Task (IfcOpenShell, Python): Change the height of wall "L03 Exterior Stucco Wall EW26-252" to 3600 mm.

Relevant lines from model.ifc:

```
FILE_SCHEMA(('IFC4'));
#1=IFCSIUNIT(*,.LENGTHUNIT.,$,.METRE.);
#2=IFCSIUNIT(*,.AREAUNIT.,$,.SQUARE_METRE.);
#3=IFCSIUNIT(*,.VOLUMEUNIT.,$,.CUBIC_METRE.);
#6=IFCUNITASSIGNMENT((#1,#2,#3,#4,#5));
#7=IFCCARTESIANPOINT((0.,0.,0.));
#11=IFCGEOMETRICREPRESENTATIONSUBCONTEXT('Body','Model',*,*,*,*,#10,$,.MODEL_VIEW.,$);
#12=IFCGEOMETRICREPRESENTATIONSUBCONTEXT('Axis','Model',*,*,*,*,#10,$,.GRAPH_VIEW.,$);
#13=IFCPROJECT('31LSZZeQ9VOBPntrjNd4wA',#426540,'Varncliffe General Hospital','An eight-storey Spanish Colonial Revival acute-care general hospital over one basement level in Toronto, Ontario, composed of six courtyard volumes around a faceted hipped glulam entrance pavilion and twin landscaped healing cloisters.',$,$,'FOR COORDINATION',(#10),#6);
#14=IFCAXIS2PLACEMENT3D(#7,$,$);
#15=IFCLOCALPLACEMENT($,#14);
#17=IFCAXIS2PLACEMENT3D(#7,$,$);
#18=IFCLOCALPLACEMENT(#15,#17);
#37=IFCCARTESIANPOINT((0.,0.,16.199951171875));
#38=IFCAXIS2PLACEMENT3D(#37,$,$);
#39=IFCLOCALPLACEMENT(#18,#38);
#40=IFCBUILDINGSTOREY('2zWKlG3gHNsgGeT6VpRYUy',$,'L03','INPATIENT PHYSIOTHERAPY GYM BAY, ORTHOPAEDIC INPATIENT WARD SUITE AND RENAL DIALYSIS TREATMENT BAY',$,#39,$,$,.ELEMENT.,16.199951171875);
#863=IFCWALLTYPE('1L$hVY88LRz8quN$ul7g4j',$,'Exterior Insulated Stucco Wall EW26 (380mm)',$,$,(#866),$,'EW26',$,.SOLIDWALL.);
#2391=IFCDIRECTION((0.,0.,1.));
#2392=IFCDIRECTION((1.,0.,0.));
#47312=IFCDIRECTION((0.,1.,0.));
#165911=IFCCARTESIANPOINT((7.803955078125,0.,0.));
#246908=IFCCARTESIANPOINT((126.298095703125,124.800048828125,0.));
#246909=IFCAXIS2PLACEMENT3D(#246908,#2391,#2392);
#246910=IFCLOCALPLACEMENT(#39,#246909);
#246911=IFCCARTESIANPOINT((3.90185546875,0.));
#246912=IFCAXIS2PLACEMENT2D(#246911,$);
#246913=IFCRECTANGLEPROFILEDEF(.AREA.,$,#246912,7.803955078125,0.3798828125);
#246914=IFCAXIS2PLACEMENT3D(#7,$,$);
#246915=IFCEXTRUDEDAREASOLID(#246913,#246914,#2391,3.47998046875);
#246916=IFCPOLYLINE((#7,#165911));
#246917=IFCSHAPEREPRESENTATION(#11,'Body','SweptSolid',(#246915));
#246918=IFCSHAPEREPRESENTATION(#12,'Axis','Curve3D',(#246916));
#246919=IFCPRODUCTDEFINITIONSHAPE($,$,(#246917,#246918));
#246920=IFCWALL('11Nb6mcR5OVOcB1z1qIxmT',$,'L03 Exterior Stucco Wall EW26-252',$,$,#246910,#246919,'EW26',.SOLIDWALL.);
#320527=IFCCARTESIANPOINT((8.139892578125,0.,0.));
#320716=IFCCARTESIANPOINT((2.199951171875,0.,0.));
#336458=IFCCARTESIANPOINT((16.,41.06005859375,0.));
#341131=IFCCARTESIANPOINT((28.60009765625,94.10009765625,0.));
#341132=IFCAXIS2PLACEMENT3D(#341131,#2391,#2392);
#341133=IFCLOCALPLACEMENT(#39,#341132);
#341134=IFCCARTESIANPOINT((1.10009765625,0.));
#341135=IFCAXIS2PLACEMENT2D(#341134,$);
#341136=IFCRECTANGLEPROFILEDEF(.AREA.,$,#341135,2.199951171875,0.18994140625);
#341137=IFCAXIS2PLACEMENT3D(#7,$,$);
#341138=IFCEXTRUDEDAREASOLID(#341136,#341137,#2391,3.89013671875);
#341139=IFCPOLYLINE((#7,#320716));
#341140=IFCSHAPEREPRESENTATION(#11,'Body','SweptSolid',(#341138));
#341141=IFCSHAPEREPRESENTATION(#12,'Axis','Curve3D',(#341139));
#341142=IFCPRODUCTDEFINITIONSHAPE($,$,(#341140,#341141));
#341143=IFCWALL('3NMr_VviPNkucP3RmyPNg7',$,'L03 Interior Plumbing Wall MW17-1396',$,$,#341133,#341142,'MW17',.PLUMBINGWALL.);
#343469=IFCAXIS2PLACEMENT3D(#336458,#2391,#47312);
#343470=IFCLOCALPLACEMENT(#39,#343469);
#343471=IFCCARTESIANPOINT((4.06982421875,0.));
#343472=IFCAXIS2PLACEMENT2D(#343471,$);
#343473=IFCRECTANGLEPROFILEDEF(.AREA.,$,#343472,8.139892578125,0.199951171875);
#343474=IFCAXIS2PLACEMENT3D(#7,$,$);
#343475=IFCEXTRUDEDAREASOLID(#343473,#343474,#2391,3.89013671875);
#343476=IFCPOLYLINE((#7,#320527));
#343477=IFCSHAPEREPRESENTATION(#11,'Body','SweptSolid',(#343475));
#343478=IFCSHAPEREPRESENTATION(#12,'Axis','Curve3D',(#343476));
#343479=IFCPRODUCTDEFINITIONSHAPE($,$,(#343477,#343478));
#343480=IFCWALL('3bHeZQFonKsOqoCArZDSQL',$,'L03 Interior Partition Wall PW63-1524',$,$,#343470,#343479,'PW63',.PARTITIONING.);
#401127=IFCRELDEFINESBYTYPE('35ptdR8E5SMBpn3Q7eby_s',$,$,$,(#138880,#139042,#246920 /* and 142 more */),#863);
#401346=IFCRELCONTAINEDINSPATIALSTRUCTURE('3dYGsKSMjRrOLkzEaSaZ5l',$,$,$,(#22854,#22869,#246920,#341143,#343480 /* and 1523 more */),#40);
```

```python
import ifcopenshell
import ifcopenshell.geom
import ifcopenshell.util.representation
import ifcopenshell.util.shape

model = ifcopenshell.open("model.ifc")
settings = ifcopenshell.geom.settings()


def volume(element):
    """Net volume in cubic metres, openings subtracted."""
    shape = ifcopenshell.geom.create_shape(settings, element)
    return ifcopenshell.util.shape.get_volume(shape.geometry)


wall = model.by_guid("11Nb6mcR5OVOcB1z1qIxmT")
before = volume(wall)

body = ifcopenshell.util.representation.get_representation(wall, "Model", "Body")
solid = body.Items[0]
old_height = solid.Depth
solid.Depth = 3.6
after = volume(wall)

print(f"height {old_height:g} -> {solid.Depth:g}, volume {before:.3f} -> {after:.3f} m3")

model.write("model-out.ifc")
```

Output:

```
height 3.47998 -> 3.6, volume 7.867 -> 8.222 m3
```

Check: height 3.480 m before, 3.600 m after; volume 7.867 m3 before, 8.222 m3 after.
